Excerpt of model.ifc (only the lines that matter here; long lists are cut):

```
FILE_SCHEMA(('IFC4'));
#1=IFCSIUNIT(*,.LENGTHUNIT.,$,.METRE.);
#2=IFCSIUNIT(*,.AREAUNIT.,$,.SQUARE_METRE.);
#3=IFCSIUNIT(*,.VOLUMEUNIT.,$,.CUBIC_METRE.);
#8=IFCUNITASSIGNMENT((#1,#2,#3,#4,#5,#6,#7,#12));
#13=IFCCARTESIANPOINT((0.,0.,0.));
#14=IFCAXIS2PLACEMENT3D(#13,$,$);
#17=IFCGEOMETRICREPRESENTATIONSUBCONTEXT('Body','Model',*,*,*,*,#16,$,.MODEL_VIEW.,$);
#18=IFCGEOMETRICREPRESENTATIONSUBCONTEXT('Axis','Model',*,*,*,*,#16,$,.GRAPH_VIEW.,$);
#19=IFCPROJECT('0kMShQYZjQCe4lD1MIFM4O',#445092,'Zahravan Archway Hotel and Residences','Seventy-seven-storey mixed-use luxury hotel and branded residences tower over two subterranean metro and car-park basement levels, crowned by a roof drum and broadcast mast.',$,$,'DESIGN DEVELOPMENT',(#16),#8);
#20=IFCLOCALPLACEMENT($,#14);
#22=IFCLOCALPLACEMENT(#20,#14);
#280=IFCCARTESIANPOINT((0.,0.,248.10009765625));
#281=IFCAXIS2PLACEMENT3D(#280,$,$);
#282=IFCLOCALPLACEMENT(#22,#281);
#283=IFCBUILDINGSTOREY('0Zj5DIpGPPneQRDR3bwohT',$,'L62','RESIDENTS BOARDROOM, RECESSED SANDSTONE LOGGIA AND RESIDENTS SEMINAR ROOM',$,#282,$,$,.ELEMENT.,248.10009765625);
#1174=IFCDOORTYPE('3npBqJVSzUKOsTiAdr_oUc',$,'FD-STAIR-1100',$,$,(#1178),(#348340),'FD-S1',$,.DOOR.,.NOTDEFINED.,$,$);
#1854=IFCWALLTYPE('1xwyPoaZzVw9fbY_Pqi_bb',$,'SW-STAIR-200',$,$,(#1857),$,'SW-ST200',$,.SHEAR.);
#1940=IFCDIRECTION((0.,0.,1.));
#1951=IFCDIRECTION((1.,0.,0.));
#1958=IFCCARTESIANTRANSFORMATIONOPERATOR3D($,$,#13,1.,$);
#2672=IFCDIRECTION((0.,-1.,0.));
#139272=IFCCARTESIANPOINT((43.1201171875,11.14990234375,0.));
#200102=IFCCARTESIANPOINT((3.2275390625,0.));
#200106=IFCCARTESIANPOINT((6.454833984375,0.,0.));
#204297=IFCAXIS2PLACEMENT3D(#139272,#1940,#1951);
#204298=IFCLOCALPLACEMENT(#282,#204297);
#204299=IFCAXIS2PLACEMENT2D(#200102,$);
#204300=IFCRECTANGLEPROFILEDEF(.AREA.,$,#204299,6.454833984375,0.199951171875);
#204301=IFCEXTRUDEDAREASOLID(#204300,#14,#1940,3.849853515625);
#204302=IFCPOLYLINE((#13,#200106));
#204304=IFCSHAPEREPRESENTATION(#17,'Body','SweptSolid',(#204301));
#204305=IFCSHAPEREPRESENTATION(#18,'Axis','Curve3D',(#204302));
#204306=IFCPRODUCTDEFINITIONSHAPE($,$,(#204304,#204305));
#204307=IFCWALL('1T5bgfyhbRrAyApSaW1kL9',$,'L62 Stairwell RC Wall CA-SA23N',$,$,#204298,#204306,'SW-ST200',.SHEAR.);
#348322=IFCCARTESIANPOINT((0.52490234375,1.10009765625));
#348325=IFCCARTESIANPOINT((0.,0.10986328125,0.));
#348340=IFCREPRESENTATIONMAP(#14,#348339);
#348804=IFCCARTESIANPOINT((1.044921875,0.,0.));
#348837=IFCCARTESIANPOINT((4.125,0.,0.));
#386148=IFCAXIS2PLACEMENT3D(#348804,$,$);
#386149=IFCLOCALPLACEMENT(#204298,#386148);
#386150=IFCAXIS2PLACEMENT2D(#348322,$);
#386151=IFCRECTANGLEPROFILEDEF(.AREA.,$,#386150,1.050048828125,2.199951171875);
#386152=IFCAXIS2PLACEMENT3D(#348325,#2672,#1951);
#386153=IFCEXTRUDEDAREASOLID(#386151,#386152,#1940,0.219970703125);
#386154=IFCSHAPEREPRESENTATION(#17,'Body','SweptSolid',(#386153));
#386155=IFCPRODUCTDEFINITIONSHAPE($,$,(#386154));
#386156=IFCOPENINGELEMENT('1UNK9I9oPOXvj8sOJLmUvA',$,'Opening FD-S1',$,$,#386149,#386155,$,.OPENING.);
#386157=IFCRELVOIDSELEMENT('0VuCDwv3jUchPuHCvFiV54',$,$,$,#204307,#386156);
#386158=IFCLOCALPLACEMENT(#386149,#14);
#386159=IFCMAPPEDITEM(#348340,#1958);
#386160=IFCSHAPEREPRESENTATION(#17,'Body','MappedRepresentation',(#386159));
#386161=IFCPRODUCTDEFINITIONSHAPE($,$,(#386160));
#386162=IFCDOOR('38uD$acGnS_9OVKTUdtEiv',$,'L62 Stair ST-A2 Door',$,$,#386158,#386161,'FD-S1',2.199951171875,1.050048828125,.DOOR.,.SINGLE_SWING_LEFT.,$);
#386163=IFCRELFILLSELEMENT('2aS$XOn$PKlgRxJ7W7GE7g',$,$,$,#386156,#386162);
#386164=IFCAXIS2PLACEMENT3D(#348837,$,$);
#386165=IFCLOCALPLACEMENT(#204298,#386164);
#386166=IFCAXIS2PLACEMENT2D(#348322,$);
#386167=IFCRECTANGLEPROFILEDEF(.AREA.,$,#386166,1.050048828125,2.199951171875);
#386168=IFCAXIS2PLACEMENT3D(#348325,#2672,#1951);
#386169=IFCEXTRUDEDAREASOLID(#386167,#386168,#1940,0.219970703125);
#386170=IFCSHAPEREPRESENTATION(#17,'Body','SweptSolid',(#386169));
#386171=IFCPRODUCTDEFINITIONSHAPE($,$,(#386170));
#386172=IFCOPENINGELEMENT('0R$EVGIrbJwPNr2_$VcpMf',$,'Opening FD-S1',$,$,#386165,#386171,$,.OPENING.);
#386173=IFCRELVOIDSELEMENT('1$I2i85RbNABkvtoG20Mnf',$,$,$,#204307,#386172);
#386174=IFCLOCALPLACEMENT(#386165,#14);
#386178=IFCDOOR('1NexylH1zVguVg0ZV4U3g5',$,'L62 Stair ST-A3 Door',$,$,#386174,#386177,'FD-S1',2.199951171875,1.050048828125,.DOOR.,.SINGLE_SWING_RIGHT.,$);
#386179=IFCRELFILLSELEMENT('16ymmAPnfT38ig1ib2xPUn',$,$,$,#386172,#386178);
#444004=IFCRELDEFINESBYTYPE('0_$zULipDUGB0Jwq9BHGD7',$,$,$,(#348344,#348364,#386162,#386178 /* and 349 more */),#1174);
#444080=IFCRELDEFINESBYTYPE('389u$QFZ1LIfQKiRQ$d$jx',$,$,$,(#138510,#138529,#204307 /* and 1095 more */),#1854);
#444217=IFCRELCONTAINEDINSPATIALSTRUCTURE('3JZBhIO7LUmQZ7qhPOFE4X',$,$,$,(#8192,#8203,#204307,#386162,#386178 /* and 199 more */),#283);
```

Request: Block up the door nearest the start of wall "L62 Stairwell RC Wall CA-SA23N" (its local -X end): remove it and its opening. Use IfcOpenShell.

```python
import ifcopenshell
import ifcopenshell.api.feature
import ifcopenshell.api.root
import ifcopenshell.geom
import ifcopenshell.util.shape

model = ifcopenshell.open("model.ifc")
settings = ifcopenshell.geom.settings()


def volume(element):
    """Net volume in cubic metres, openings subtracted."""
    shape = ifcopenshell.geom.create_shape(settings, element)
    return ifcopenshell.util.shape.get_volume(shape.geometry)


door = model.by_guid("38uD$acGnS_9OVKTUdtEiv")
opening = door.FillsVoids[0].RelatingOpeningElement
wall = opening.VoidsElements[0].RelatingBuildingElement
before = volume(wall)

ifcopenshell.api.root.remove_product(model, product=door)
ifcopenshell.api.feature.remove_feature(model, feature=opening)

after = volume(wall)

print(f"wall volume {before:.3f} -> {after:.3f} m3")

model.write("model_edited.ifc")
```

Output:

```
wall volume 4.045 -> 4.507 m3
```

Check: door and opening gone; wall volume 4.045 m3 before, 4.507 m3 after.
